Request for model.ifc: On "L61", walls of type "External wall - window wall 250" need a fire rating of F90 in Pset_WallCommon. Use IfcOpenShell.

First a look at what the model holds.

```python
import ifcopenshell
import ifcopenshell.util.element

model = ifcopenshell.open("model.ifc")
print(model.schema)
storey = next(s for s in model.by_type("IfcBuildingStorey") if s.Name == "L61")
walls = [e for e in ifcopenshell.util.element.get_decomposition(storey) if e.is_a("IfcWall")]
seen = {}
for e in walls:
    element_type = ifcopenshell.util.element.get_type(e)
    key = (element_type.Name if element_type != e and element_type else None, ifcopenshell.util.element.get_pset(e, "Pset_WallCommon", "FireRating"))
    seen[key] = seen.get(key, 0) + 1
for (name, value), count in sorted(seen.items(), key=str):
    print(count, "x", name, "|", value)
```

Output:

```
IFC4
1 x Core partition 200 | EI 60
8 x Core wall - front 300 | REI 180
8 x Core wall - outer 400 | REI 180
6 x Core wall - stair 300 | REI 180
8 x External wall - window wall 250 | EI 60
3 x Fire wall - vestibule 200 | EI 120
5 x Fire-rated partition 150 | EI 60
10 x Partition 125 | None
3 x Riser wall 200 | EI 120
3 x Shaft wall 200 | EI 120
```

```python
import ifcopenshell
import ifcopenshell.api.pset
import ifcopenshell.util.element

model = ifcopenshell.open("model.ifc")

storey = next(s for s in model.by_type("IfcBuildingStorey") if s.Name == "L61")
walls = [e for e in ifcopenshell.util.element.get_decomposition(storey) if e.is_a("IfcWall")]

count = 0
for e in walls:
    element_type = ifcopenshell.util.element.get_type(e)
    if element_type in (None, e) or element_type.Name != "External wall - window wall 250":
        continue
    found = ifcopenshell.util.element.get_pset(e, "Pset_WallCommon", should_inherit=False)
    if found:
        pset = model.by_id(found["id"])
        if len(ifcopenshell.util.element.get_elements_by_pset(pset)) > 1:
            pset = ifcopenshell.api.pset.unshare_pset(model, products=[e], pset=pset)[0]
    else:
        pset = ifcopenshell.api.pset.add_pset(model, product=e, name="Pset_WallCommon")
    ifcopenshell.api.pset.edit_pset(model, pset=pset, properties={"FireRating": "F90"})
    count += 1

print(count, "walls updated")

model.write("model_rev.ifc")
```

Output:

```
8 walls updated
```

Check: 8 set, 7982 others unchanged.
